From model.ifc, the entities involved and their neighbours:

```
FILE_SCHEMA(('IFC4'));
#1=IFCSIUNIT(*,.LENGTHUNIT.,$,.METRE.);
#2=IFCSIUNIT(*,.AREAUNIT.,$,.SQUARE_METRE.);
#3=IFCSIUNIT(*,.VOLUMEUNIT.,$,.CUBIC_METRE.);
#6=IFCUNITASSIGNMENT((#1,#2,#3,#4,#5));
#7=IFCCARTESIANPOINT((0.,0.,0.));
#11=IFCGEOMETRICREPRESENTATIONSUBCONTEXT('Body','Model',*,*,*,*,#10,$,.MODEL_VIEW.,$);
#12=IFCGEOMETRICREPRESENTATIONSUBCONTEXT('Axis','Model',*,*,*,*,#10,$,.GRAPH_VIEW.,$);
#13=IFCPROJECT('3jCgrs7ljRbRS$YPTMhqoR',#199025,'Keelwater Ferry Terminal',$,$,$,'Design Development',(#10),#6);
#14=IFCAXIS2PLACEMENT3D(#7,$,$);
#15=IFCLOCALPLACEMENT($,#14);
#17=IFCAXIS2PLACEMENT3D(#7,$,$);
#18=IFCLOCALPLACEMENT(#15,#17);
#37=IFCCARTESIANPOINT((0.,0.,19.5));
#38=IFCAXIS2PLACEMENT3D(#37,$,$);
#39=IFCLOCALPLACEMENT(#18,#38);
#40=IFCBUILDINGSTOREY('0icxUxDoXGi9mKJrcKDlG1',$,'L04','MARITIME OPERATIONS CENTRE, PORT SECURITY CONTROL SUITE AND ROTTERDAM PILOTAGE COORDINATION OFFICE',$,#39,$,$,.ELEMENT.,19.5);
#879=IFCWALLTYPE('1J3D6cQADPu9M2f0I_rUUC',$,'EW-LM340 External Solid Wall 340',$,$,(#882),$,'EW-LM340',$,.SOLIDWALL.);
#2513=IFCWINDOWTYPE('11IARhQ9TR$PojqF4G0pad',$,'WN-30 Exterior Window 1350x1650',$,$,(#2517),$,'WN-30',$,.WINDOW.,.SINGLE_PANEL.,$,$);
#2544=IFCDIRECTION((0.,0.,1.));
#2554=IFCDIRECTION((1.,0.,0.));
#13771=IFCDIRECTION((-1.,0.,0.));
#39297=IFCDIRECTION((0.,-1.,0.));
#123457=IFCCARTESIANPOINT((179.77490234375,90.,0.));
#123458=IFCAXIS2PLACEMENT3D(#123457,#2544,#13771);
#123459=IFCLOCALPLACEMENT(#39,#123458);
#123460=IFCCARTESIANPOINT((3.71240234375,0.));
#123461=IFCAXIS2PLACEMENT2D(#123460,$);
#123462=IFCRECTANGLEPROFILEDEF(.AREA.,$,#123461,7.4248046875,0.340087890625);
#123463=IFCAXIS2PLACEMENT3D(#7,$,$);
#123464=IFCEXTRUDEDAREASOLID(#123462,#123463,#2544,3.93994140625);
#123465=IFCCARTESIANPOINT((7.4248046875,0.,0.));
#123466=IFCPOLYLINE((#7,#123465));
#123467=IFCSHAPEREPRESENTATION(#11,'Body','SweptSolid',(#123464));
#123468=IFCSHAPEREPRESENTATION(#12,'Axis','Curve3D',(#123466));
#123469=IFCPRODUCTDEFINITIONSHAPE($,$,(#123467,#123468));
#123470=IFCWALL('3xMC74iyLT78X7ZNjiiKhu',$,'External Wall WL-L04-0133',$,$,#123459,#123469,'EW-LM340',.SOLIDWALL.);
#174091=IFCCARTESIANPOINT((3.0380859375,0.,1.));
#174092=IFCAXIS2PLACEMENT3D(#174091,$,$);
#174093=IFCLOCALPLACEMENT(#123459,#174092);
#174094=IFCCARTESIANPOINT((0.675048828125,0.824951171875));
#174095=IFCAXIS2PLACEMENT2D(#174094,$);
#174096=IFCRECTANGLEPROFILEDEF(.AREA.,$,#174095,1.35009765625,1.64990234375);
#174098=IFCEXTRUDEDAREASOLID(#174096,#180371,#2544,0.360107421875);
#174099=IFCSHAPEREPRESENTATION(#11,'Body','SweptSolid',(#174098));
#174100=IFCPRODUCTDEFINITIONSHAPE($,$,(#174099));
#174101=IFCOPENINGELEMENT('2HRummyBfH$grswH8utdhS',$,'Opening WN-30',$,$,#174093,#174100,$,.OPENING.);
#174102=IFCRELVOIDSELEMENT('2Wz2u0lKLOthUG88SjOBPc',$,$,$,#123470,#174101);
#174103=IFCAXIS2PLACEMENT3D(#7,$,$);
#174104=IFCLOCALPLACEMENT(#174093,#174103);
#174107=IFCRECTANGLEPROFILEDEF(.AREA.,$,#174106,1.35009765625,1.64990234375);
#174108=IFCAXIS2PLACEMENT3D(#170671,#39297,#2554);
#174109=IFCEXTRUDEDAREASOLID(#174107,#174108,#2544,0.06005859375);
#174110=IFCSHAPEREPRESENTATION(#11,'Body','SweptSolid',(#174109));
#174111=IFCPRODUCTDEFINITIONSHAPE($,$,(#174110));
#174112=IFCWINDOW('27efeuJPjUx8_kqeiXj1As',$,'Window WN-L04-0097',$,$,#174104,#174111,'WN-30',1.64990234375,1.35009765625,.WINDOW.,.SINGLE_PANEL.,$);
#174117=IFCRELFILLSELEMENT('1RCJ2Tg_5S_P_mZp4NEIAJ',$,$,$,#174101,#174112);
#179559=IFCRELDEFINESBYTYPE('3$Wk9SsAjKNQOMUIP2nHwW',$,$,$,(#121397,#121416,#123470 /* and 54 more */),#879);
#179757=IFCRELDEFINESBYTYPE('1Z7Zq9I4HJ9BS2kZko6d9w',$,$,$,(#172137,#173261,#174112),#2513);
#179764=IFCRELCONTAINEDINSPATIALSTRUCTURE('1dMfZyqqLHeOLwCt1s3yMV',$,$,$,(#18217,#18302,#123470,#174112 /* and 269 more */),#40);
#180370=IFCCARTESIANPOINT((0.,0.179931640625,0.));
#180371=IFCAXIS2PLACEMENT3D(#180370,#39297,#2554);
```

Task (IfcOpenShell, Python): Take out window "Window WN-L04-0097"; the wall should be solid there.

```python
import ifcopenshell
import ifcopenshell.api.feature
import ifcopenshell.api.root
import ifcopenshell.geom
import ifcopenshell.util.shape

model = ifcopenshell.open("model.ifc")
settings = ifcopenshell.geom.settings()


def volume(element):
    """Net volume in cubic metres, openings subtracted."""
    shape = ifcopenshell.geom.create_shape(settings, element)
    return ifcopenshell.util.shape.get_volume(shape.geometry)


window = model.by_id(174112)
opening = window.FillsVoids[0].RelatingOpeningElement
wall = opening.VoidsElements[0].RelatingBuildingElement
before = volume(wall)

ifcopenshell.api.root.remove_product(model, product=window)
ifcopenshell.api.feature.remove_feature(model, feature=opening)

after = volume(wall)

print(f"wall volume {before:.3f} -> {after:.3f} m3")

model.write("model_v2.ifc")
```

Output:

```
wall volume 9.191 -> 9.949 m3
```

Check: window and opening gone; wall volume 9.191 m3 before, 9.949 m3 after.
